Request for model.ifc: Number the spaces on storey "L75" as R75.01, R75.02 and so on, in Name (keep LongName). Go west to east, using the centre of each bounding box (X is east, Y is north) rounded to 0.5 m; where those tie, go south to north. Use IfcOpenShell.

First a look at what the model holds.

```python
import ifcopenshell
import ifcopenshell.util.element
import ifcopenshell.util.placement

model = ifcopenshell.open("model.ifc")
print(model.schema)
storey = next(s for s in model.by_type("IfcBuildingStorey") if s.Name == "L75")
spaces = [e for e in ifcopenshell.util.element.get_decomposition(storey) if e.is_a("IfcSpace")]
for e in sorted(spaces, key=lambda e: e.id()):
    origin = ifcopenshell.util.placement.get_local_placement(e.ObjectPlacement)[:3, 3]
    print(e.id(), e.Name, e.LongName, origin.round(2) + 0.0, sep=" | ")
```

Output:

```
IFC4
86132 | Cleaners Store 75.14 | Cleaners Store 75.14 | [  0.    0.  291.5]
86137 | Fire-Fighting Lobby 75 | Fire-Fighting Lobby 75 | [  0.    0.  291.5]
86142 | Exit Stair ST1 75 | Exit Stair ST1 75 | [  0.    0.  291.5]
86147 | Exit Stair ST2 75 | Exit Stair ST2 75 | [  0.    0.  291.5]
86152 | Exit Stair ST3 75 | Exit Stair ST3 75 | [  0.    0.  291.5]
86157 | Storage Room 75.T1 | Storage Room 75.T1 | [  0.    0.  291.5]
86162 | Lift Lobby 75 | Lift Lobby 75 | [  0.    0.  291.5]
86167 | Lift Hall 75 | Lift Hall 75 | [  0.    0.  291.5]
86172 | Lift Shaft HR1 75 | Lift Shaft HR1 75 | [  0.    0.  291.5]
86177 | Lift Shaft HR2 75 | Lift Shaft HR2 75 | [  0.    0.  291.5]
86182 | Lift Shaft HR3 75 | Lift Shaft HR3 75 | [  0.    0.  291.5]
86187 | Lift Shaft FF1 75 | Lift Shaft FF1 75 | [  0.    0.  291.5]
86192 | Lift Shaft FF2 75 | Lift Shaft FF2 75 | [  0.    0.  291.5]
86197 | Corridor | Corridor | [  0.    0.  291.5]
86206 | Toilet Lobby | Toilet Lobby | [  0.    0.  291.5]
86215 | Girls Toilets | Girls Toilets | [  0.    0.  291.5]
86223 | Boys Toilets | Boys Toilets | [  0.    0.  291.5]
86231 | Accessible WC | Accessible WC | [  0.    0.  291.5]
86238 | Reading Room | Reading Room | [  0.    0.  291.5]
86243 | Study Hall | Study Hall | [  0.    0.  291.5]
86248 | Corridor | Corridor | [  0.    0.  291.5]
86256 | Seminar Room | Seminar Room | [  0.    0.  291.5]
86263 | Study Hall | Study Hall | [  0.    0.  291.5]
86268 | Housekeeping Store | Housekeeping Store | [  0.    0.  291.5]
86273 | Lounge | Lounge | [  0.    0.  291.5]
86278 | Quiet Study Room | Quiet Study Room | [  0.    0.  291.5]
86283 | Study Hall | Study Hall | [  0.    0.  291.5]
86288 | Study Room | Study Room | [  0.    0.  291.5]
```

```python
import ifcopenshell
import ifcopenshell.geom
import ifcopenshell.util.element
import ifcopenshell.util.shape

model = ifcopenshell.open("model.ifc")
settings = ifcopenshell.geom.settings()
settings.set("use-world-coords", True)


def centre(element):
    shape = ifcopenshell.geom.create_shape(settings, element)
    return ifcopenshell.util.shape.get_bbox_centroid(shape.geometry)


storey = next(s for s in model.by_type("IfcBuildingStorey") if s.Name == "L75")
spaces = [e for e in ifcopenshell.util.element.get_decomposition(storey) if e.is_a("IfcSpace")]

# Insertion points can sit at a corner or the storey origin, so sort by the geometry (in metres).
centres = {e: centre(e) for e in spaces}
spaces.sort(key=lambda e: (round(centres[e][0] / 0.5), centres[e][1]))

for i, e in enumerate(spaces, start=1):
    number = f"R75.{i:02d}"
    e.Name = number
    print(e.id(), number)

model.write("model_edited.ifc")
```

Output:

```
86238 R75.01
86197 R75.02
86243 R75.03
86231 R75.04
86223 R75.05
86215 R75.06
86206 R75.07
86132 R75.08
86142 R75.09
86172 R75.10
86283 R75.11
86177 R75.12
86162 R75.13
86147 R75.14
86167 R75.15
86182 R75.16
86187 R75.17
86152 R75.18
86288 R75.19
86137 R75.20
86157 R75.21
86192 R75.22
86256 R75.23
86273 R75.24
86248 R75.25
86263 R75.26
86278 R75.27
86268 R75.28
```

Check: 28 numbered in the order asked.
